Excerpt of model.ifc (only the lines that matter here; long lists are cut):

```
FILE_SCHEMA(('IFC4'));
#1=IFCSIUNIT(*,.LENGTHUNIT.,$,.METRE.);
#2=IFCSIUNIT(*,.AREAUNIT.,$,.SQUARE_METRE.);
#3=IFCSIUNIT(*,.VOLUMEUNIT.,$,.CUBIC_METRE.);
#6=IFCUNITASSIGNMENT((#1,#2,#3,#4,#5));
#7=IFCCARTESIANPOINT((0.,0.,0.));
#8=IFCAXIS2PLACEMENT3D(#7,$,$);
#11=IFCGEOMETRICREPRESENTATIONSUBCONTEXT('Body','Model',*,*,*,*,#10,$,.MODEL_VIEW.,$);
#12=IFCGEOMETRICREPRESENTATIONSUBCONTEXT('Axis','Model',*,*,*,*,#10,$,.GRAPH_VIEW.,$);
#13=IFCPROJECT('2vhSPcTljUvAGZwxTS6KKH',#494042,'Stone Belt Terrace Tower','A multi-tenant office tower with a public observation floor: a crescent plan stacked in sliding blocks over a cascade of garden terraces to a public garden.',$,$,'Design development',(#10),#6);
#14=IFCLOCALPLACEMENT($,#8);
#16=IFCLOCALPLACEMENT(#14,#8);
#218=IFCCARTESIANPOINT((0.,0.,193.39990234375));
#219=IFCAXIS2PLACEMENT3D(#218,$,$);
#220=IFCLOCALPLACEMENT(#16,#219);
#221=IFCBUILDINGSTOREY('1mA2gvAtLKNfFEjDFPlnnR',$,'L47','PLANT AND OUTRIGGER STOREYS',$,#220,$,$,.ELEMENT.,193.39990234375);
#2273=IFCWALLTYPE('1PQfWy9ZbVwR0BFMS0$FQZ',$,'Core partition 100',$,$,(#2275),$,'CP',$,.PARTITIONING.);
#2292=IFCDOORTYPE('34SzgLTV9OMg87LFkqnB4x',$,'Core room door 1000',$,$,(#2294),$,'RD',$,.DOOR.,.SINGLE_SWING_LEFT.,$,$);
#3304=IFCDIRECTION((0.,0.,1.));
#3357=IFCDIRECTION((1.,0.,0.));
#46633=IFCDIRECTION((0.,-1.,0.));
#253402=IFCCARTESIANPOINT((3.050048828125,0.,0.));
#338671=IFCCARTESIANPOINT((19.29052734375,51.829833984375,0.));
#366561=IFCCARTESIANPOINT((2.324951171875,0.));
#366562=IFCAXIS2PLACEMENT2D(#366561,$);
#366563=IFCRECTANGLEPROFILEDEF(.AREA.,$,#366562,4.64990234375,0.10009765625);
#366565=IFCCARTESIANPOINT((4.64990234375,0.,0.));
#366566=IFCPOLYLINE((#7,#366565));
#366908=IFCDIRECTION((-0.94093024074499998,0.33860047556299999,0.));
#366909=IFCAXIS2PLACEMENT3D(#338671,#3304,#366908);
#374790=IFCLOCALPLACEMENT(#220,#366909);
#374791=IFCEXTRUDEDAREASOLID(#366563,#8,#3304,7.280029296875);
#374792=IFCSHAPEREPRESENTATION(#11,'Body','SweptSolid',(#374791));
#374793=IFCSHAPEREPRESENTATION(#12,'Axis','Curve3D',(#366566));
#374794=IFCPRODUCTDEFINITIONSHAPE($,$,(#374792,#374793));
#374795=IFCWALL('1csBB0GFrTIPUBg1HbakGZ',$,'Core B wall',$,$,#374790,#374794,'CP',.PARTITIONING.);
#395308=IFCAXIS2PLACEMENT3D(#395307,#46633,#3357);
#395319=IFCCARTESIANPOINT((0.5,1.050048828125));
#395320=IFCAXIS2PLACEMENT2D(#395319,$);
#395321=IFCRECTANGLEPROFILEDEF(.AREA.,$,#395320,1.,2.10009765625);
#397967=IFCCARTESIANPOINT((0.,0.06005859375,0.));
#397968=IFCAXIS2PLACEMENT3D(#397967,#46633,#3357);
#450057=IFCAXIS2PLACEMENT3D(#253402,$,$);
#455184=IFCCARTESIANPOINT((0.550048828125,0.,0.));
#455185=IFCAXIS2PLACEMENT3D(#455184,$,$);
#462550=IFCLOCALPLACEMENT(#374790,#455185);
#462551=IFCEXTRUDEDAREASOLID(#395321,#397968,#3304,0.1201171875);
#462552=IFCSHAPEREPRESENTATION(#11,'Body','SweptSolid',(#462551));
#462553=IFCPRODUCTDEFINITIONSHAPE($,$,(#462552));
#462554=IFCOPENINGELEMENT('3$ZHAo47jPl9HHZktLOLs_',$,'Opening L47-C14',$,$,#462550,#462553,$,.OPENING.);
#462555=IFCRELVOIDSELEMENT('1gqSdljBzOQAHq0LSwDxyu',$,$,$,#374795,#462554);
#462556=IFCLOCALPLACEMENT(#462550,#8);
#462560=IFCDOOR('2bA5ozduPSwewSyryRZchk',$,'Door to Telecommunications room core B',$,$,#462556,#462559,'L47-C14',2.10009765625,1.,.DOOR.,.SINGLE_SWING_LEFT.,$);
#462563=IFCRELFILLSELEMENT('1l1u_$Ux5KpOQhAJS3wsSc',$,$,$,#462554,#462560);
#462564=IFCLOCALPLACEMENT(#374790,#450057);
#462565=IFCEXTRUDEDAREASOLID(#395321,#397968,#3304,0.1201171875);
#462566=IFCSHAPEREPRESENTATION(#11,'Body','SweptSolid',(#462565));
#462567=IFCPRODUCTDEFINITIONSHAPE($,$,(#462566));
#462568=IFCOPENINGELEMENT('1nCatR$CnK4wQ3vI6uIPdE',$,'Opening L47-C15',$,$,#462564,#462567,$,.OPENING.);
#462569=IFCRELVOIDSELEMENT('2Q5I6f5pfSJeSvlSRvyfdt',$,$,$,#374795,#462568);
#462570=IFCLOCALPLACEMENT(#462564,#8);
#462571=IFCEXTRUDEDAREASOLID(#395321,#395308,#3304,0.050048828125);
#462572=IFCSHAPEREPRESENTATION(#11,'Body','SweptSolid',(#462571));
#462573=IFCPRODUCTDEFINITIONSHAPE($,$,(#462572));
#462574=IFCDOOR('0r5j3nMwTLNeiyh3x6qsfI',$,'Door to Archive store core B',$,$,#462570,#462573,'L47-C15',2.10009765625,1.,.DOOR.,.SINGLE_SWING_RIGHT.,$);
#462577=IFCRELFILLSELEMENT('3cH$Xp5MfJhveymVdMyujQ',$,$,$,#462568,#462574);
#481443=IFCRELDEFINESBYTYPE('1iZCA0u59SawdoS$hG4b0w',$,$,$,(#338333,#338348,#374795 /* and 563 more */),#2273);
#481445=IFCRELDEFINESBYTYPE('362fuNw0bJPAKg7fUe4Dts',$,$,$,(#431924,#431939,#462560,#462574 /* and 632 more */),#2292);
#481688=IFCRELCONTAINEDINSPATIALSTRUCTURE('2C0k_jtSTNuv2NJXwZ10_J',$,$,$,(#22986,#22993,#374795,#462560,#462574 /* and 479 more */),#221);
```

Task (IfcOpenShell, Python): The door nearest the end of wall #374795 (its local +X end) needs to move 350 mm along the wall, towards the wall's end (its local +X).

```python
import ifcopenshell
import ifcopenshell.api.geometry
import ifcopenshell.util.placement

model = ifcopenshell.open("model.ifc")

door = model.by_guid("0r5j3nMwTLNeiyh3x6qsfI")
opening = door.FillsVoids[0].RelatingOpeningElement
wall = opening.VoidsElements[0].RelatingBuildingElement

wall_matrix = ifcopenshell.util.placement.get_local_placement(wall.ObjectPlacement)
shift = wall_matrix[:3, 0] * 0.35
before = ifcopenshell.util.placement.get_local_placement(door.ObjectPlacement)[:3, 3].copy()

# The door is placed relative to its opening, so it follows when the opening moves.
matrix = ifcopenshell.util.placement.get_local_placement(opening.ObjectPlacement)
matrix[:3, 3] += shift
ifcopenshell.api.geometry.edit_object_placement(
    model, product=opening, matrix=matrix, is_si=False, should_transform_children=True
)

after = ifcopenshell.util.placement.get_local_placement(door.ObjectPlacement)[:3, 3]
print("door moved by", (after - before).round(3) + 0.0)

model.write("model_edited.ifc")
```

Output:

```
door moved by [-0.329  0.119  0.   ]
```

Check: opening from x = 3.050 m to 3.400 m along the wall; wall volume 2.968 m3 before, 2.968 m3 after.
